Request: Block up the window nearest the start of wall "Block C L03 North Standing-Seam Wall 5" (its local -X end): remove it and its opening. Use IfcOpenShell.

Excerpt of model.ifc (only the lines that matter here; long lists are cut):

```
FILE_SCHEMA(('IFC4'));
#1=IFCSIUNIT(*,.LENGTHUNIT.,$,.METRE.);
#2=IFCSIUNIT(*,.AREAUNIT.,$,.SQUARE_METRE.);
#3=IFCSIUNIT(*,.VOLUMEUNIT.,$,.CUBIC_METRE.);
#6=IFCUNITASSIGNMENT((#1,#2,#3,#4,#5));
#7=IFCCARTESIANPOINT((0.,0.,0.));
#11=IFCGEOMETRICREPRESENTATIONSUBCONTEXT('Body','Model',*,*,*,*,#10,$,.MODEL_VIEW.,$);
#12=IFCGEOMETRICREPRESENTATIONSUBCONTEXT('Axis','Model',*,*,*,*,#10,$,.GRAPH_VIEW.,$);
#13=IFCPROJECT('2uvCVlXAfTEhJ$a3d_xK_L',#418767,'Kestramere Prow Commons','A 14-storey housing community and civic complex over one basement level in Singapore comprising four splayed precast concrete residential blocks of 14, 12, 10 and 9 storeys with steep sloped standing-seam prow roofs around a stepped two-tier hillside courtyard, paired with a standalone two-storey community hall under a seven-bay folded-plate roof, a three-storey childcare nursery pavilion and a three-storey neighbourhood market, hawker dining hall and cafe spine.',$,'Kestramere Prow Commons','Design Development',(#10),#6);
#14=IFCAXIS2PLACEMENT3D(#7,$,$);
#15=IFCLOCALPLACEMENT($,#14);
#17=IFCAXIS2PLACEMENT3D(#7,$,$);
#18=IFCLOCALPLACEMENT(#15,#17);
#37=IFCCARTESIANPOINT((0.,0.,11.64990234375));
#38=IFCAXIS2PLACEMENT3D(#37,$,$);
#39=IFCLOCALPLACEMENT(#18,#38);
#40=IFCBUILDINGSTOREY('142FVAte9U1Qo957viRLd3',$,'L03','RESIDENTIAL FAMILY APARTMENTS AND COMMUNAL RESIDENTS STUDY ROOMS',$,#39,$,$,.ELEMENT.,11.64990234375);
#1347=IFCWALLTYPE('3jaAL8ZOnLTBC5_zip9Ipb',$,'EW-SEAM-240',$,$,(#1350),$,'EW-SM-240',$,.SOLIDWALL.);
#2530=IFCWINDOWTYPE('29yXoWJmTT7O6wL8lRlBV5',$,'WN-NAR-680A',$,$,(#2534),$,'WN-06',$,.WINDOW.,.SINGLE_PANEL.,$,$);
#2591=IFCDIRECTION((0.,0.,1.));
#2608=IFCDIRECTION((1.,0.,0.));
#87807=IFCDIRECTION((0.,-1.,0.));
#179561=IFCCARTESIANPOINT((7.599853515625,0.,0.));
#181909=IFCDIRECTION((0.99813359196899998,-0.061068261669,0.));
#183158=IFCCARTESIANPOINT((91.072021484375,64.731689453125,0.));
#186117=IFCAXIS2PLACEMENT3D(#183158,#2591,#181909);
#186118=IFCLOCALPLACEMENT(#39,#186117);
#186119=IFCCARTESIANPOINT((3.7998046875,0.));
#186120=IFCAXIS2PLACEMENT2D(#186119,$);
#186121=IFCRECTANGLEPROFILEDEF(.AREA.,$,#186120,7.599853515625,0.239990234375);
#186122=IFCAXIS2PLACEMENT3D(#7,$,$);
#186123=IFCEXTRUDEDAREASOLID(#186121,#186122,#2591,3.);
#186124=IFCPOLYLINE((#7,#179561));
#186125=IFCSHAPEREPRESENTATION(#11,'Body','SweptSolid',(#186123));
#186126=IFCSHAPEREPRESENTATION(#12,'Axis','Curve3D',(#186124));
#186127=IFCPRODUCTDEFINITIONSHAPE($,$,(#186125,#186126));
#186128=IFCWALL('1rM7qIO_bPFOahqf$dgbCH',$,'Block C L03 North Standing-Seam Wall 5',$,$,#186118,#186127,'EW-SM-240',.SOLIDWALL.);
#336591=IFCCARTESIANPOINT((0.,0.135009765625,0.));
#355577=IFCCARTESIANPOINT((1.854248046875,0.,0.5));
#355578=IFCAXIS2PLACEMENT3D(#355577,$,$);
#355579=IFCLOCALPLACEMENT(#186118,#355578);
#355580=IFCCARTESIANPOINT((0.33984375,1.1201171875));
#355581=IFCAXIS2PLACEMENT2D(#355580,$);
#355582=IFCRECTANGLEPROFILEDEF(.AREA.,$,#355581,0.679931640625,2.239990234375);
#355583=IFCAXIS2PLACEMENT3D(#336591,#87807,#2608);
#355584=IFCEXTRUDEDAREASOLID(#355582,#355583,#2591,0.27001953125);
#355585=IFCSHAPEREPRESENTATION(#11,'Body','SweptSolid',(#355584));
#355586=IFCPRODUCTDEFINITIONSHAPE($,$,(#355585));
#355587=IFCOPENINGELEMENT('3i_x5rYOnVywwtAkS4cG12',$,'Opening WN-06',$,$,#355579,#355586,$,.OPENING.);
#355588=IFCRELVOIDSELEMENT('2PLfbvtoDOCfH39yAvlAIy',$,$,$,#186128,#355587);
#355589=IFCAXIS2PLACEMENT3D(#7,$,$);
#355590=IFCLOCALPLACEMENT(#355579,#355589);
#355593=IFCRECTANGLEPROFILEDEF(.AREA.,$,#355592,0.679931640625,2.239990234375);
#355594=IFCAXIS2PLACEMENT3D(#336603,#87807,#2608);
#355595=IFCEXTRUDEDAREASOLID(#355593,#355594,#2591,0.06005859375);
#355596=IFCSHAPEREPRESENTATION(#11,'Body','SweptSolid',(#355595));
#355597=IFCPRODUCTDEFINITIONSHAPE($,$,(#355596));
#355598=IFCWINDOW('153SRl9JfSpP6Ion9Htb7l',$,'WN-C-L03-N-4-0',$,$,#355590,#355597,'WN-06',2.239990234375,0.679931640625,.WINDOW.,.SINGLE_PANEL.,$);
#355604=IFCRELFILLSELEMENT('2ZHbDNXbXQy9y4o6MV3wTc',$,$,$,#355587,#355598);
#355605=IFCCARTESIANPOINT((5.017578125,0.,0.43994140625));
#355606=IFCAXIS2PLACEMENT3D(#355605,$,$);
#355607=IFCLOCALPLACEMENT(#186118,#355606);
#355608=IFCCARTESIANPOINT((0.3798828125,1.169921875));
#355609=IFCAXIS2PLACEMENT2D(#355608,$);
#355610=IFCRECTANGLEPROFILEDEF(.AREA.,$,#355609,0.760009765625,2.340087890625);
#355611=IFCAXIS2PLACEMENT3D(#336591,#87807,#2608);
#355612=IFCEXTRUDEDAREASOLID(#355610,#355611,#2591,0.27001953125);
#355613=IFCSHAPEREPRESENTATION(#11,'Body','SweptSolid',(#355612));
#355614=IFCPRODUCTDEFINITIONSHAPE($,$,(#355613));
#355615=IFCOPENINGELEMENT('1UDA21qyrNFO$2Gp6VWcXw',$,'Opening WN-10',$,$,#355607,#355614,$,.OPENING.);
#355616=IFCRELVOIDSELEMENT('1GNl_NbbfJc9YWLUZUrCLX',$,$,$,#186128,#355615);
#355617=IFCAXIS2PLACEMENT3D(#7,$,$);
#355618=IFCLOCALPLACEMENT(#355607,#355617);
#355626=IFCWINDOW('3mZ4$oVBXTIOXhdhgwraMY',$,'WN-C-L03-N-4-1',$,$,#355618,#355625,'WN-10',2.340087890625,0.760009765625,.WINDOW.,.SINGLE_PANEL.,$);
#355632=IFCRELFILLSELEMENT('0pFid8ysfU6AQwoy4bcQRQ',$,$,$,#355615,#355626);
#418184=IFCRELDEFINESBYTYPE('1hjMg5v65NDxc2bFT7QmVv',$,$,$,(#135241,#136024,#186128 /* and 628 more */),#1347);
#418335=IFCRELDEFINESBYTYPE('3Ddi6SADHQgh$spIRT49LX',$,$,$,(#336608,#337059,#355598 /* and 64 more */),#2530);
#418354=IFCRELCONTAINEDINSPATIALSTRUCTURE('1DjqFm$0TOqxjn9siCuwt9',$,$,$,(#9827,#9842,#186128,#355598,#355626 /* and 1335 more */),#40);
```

```python
import ifcopenshell
import ifcopenshell.api.feature
import ifcopenshell.api.root
import ifcopenshell.geom
import ifcopenshell.util.shape

model = ifcopenshell.open("model.ifc")
settings = ifcopenshell.geom.settings()


def volume(element):
    """Net volume in cubic metres, openings subtracted."""
    shape = ifcopenshell.geom.create_shape(settings, element)
    return ifcopenshell.util.shape.get_volume(shape.geometry)


window = model.by_guid("153SRl9JfSpP6Ion9Htb7l")
opening = window.FillsVoids[0].RelatingOpeningElement
wall = opening.VoidsElements[0].RelatingBuildingElement
before = volume(wall)

ifcopenshell.api.root.remove_product(model, product=window)
ifcopenshell.api.feature.remove_feature(model, feature=opening)

after = volume(wall)

print(f"wall volume {before:.3f} -> {after:.3f} m3")

model.write("model_updated.ifc")
```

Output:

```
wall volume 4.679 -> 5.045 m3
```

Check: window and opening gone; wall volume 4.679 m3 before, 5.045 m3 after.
